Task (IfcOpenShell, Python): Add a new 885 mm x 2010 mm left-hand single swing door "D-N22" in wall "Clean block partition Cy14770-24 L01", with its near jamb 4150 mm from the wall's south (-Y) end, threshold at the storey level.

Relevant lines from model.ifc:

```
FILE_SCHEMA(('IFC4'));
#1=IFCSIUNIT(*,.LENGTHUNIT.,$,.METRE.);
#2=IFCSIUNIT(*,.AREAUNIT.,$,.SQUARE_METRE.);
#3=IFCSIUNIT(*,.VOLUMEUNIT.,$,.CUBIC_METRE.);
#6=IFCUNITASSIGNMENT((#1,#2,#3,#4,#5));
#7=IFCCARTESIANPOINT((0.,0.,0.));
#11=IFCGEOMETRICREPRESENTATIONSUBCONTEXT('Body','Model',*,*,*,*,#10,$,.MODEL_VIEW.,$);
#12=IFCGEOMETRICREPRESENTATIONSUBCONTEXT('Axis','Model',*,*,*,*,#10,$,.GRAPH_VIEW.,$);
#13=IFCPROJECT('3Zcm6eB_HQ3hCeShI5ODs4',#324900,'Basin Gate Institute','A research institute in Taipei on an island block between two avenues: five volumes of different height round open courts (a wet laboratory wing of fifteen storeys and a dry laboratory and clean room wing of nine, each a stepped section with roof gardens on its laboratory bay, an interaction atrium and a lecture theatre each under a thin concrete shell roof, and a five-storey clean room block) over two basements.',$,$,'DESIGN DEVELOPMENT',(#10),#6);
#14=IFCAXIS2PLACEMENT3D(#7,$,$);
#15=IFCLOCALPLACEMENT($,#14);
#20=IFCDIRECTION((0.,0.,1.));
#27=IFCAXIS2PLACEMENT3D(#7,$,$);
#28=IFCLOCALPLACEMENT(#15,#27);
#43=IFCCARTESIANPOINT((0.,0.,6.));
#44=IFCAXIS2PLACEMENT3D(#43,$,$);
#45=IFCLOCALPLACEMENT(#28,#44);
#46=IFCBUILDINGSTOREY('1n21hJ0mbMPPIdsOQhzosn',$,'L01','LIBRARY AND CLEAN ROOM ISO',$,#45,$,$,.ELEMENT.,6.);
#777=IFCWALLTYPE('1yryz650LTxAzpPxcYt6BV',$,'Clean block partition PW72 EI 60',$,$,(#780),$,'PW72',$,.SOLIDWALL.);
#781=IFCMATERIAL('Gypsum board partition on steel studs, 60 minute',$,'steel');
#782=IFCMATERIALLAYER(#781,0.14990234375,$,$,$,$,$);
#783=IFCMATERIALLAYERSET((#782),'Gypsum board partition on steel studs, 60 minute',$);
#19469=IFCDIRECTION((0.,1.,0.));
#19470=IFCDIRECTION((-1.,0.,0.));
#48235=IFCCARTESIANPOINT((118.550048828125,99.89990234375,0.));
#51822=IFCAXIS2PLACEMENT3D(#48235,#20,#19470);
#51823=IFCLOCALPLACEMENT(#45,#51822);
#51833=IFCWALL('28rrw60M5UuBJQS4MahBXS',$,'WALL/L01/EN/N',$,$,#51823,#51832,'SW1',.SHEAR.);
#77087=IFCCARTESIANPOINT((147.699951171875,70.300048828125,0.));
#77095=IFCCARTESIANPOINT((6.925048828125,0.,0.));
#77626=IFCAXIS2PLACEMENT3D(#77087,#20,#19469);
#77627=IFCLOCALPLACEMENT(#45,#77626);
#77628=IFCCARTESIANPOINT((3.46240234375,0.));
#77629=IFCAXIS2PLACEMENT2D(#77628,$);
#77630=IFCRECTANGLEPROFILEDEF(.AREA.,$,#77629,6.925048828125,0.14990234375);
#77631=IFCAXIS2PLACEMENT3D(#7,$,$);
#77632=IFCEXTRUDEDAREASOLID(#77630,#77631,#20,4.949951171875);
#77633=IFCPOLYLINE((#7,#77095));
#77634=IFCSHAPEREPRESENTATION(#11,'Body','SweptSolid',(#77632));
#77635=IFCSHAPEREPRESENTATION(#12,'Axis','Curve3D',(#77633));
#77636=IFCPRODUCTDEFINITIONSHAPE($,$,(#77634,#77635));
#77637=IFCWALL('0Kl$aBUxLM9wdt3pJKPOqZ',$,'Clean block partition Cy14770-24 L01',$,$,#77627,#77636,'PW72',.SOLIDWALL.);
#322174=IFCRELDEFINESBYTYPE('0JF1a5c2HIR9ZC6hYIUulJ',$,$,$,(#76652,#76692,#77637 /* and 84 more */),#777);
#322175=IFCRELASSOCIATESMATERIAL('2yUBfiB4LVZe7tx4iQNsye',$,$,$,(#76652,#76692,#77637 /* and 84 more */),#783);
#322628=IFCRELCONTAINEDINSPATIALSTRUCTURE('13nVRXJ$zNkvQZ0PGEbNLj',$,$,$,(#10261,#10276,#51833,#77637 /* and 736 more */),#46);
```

```python
import numpy as np
import ifcopenshell
import ifcopenshell.api.feature
import ifcopenshell.api.geometry
import ifcopenshell.api.root
import ifcopenshell.api.spatial
import ifcopenshell.geom
import ifcopenshell.util.element
import ifcopenshell.util.placement
import ifcopenshell.util.representation
import ifcopenshell.util.shape
import ifcopenshell.util.unit

model = ifcopenshell.open("model.ifc")
unit_scale = ifcopenshell.util.unit.calculate_unit_scale(model)
settings = ifcopenshell.geom.settings()


def volume(element):
    """Net volume in cubic metres, openings subtracted."""
    shape = ifcopenshell.geom.create_shape(settings, element)
    return ifcopenshell.util.shape.get_volume(shape.geometry)


wall = model.by_id(77637)
storey = ifcopenshell.util.element.get_container(wall, ifc_class="IfcBuildingStorey")
context = ifcopenshell.util.representation.get_context(model, "Model", "Body", "MODEL_VIEW")
before = volume(wall)

width, height, from_end, sill = 0.885, 2.01, 4.15, 0.0  # metres

# The wall runs along its own X axis, and the end named is its -X end.
wall_shape = ifcopenshell.geom.create_shape(settings, wall)
x, y, z = ifcopenshell.util.shape.get_vertices(wall_shape.geometry).T
start = x.min() + from_end
face, thickness = float(y.min()), float(y.max() - y.min())
wall_matrix = ifcopenshell.util.placement.get_local_placement(wall.ObjectPlacement)
level = ifcopenshell.util.placement.get_local_placement(storey.ObjectPlacement)[2, 3]


def in_wall(x, y):
    """Placement at x, y metres in the wall's axes, at sill height."""
    matrix = wall_matrix.copy()
    matrix[:, 3] = wall_matrix @ np.array([x / unit_scale, y / unit_scale, 0.0, 1.0])
    matrix[2, 3] = level + sill / unit_scale
    return matrix


# Opening: a box that overshoots both wall faces by 50 mm.
opening = ifcopenshell.api.root.create_entity(model, ifc_class="IfcOpeningElement", predefined_type="OPENING")
box = ifcopenshell.api.geometry.add_wall_representation(
    model, context=context, length=width, height=height, thickness=thickness + 0.1
)
ifcopenshell.api.geometry.assign_representation(model, product=opening, representation=box)
ifcopenshell.api.geometry.edit_object_placement(model, product=opening, matrix=in_wall(start, face - 0.05), is_si=False)
ifcopenshell.api.feature.add_feature(model, feature=opening, element=wall)

door = ifcopenshell.api.root.create_entity(model, ifc_class="IfcDoor", name="D-N22", predefined_type="DOOR")
door.OverallWidth, door.OverallHeight = width / unit_scale, height / unit_scale
door.OperationType = "SINGLE_SWING_LEFT"
body = ifcopenshell.api.geometry.add_door_representation(
    model,
    context=context,
    overall_width=door.OverallWidth,
    overall_height=door.OverallHeight,
    operation_type="SINGLE_SWING_LEFT",
    lining_properties={"LiningDepth": thickness / unit_scale, "ThresholdDepth": thickness / unit_scale},
)
ifcopenshell.api.geometry.assign_representation(model, product=door, representation=body)
ifcopenshell.api.spatial.assign_container(model, products=[door], relating_structure=storey)
ifcopenshell.api.feature.add_filling(model, opening=opening, element=door)

# The lining spans the wall, so the door starts at the wall face.
ifcopenshell.api.geometry.edit_object_placement(model, product=door, matrix=in_wall(start, face), is_si=False)

after = volume(wall)

print(f"wall volume {before:.3f} -> {after:.3f} m3")

model.write("model_v2.ifc")
```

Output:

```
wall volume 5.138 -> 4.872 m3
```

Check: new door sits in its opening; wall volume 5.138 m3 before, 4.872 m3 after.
